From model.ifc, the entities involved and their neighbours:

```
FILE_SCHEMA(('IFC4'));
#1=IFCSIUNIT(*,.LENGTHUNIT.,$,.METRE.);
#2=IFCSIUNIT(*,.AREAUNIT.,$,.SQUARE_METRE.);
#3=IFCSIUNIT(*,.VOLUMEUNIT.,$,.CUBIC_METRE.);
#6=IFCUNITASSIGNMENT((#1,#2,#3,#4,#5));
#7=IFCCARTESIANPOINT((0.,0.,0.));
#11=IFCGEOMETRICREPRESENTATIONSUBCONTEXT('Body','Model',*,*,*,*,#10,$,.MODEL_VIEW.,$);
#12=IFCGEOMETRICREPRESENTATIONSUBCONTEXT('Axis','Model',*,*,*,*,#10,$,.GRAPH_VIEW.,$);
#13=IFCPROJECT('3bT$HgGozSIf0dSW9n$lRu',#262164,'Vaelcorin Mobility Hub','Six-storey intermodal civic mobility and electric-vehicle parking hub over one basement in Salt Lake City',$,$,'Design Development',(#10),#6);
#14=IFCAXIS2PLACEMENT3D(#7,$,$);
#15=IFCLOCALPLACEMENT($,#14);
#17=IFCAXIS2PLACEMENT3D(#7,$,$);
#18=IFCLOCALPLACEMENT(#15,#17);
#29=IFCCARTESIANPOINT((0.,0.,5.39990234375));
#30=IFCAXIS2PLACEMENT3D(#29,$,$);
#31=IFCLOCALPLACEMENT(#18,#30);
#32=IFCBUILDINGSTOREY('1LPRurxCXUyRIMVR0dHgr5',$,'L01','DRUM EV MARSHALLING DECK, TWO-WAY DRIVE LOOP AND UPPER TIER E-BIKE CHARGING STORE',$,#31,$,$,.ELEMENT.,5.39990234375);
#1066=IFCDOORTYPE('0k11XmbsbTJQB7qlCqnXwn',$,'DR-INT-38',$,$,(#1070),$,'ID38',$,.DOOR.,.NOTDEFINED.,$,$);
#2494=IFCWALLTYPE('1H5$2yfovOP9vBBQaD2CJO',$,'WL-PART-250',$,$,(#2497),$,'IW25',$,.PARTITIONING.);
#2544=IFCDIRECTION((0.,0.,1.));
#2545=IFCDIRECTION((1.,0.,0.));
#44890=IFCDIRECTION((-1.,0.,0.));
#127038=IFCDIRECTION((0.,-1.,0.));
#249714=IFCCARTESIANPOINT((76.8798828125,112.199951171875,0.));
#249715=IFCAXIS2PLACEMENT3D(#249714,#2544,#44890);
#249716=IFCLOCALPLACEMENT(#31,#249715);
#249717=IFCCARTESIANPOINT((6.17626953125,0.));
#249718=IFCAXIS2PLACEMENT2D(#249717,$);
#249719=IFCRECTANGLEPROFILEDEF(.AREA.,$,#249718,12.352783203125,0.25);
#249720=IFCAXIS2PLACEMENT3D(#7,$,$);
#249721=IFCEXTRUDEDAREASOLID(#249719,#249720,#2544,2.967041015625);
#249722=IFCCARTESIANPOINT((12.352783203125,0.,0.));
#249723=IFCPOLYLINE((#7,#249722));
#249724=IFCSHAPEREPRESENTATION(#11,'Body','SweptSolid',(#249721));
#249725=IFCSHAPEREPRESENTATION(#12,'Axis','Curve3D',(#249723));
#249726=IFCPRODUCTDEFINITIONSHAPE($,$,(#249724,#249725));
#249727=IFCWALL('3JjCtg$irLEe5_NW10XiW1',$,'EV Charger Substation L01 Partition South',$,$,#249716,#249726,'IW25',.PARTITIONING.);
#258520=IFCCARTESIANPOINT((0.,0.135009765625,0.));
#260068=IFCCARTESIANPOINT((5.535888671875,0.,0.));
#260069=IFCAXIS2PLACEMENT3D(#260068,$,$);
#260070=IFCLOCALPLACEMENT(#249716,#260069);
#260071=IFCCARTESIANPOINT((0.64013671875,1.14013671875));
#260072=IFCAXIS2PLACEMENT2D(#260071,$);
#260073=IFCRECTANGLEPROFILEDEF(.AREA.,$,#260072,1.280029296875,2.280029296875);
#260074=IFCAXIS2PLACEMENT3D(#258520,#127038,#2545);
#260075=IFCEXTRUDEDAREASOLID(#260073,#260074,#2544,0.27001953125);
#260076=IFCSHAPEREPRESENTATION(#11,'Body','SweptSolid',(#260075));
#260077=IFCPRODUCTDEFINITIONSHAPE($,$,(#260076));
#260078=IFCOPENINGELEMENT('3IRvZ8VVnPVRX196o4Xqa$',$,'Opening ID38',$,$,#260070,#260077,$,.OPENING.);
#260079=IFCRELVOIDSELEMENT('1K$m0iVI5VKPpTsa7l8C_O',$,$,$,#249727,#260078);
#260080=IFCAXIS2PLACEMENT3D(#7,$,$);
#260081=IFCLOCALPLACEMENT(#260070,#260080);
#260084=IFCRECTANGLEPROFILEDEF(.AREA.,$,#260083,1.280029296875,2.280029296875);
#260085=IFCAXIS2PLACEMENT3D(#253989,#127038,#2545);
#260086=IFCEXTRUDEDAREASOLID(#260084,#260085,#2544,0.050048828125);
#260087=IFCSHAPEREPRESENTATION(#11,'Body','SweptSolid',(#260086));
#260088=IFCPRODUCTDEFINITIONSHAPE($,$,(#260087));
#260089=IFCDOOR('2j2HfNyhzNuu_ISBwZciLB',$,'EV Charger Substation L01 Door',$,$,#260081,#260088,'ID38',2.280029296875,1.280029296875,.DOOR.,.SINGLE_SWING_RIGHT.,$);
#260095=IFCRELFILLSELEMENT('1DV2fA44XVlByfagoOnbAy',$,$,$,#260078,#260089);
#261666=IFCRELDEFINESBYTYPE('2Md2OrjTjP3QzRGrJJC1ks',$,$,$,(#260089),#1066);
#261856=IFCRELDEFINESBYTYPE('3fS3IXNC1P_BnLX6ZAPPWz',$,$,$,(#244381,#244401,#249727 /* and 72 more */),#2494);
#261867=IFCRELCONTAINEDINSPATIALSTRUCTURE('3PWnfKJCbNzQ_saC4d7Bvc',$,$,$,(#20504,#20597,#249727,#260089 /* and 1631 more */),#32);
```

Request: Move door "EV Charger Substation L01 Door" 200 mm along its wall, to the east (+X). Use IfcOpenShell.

```python
import ifcopenshell
import ifcopenshell.api.geometry
import ifcopenshell.util.placement

model = ifcopenshell.open("model.ifc")

door = model.by_guid("2j2HfNyhzNuu_ISBwZciLB")
opening = door.FillsVoids[0].RelatingOpeningElement
wall = opening.VoidsElements[0].RelatingBuildingElement

wall_matrix = ifcopenshell.util.placement.get_local_placement(wall.ObjectPlacement)
shift = wall_matrix[:3, 0] * -0.2
before = ifcopenshell.util.placement.get_local_placement(door.ObjectPlacement)[:3, 3].copy()

# The door is placed relative to its opening, so it follows when the opening moves.
matrix = ifcopenshell.util.placement.get_local_placement(opening.ObjectPlacement)
matrix[:3, 3] += shift
ifcopenshell.api.geometry.edit_object_placement(
    model, product=opening, matrix=matrix, is_si=False, should_transform_children=True
)

after = ifcopenshell.util.placement.get_local_placement(door.ObjectPlacement)[:3, 3]
print("door moved by", (after - before).round(3) + 0.0)

model.write("model_rev.ifc")
```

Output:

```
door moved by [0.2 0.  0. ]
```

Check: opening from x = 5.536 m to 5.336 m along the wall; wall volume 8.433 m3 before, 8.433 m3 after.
